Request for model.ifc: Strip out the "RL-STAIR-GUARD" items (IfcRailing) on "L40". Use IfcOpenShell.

First a look at what the model holds.

```python
import ifcopenshell
import ifcopenshell.util.element

model = ifcopenshell.open("model.ifc")
print(model.schema)
storey = next(s for s in model.by_type("IfcBuildingStorey") if s.Name == "L40")
railings = [e for e in ifcopenshell.util.element.get_decomposition(storey) if e.is_a("IfcRailing")]
seen = {}
for e in railings:
    element_type = ifcopenshell.util.element.get_type(e)
    name = element_type.Name if element_type not in (None, e) else None
    seen[name] = seen.get(name, 0) + 1
for name, count in sorted(seen.items(), key=str):
    print(count, "x", name)
```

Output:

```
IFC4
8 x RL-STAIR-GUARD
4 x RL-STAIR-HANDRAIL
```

```python
import ifcopenshell
import ifcopenshell.api.root
import ifcopenshell.util.element

model = ifcopenshell.open("model.ifc")

storey = next(s for s in model.by_type("IfcBuildingStorey") if s.Name == "L40")
railings = [e for e in ifcopenshell.util.element.get_decomposition(storey) if e.is_a("IfcRailing")]
targets = [e for e in railings if (t := ifcopenshell.util.element.get_type(e)) not in (None, e) and t.Name == "RL-STAIR-GUARD"]

for e in targets:
    ifcopenshell.api.root.remove_product(model, product=e)
print(len(targets), "removed")

model.write("model_v2.ifc")
```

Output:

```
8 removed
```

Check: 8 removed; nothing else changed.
